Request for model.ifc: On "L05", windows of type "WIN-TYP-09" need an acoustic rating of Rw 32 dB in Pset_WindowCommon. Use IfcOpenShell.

First a look at what the model holds.

```python
import ifcopenshell
import ifcopenshell.util.element

model = ifcopenshell.open("model.ifc")
print(model.schema)
storey = next(s for s in model.by_type("IfcBuildingStorey") if s.Name == "L05")
windows = [e for e in ifcopenshell.util.element.get_decomposition(storey) if e.is_a("IfcWindow")]
seen = {}
for e in windows:
    element_type = ifcopenshell.util.element.get_type(e)
    key = (element_type.Name if element_type != e and element_type else None, ifcopenshell.util.element.get_pset(e, "Pset_WindowCommon", "AcousticRating"))
    seen[key] = seen.get(key, 0) + 1
for (name, value), count in sorted(seen.items(), key=str):
    print(count, "x", name, "|", value)
```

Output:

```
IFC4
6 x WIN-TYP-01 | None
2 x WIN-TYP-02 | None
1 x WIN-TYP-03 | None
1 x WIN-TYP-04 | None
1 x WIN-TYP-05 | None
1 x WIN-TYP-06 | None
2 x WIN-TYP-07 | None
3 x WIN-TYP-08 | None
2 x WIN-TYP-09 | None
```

```python
import ifcopenshell
import ifcopenshell.api.pset
import ifcopenshell.util.element

model = ifcopenshell.open("model.ifc")

storey = next(s for s in model.by_type("IfcBuildingStorey") if s.Name == "L05")
windows = [e for e in ifcopenshell.util.element.get_decomposition(storey) if e.is_a("IfcWindow")]

count = 0
for e in windows:
    element_type = ifcopenshell.util.element.get_type(e)
    if element_type in (None, e) or element_type.Name != "WIN-TYP-09":
        continue
    # add_pset returns the element's existing set when there is one.
    pset = ifcopenshell.api.pset.add_pset(model, product=e, name="Pset_WindowCommon")
    ifcopenshell.api.pset.edit_pset(model, pset=pset, properties={"AcousticRating": "Rw 32 dB"})
    count += 1

print(count, "windows updated")

model.write("model_edited.ifc")
```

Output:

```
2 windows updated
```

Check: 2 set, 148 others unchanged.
